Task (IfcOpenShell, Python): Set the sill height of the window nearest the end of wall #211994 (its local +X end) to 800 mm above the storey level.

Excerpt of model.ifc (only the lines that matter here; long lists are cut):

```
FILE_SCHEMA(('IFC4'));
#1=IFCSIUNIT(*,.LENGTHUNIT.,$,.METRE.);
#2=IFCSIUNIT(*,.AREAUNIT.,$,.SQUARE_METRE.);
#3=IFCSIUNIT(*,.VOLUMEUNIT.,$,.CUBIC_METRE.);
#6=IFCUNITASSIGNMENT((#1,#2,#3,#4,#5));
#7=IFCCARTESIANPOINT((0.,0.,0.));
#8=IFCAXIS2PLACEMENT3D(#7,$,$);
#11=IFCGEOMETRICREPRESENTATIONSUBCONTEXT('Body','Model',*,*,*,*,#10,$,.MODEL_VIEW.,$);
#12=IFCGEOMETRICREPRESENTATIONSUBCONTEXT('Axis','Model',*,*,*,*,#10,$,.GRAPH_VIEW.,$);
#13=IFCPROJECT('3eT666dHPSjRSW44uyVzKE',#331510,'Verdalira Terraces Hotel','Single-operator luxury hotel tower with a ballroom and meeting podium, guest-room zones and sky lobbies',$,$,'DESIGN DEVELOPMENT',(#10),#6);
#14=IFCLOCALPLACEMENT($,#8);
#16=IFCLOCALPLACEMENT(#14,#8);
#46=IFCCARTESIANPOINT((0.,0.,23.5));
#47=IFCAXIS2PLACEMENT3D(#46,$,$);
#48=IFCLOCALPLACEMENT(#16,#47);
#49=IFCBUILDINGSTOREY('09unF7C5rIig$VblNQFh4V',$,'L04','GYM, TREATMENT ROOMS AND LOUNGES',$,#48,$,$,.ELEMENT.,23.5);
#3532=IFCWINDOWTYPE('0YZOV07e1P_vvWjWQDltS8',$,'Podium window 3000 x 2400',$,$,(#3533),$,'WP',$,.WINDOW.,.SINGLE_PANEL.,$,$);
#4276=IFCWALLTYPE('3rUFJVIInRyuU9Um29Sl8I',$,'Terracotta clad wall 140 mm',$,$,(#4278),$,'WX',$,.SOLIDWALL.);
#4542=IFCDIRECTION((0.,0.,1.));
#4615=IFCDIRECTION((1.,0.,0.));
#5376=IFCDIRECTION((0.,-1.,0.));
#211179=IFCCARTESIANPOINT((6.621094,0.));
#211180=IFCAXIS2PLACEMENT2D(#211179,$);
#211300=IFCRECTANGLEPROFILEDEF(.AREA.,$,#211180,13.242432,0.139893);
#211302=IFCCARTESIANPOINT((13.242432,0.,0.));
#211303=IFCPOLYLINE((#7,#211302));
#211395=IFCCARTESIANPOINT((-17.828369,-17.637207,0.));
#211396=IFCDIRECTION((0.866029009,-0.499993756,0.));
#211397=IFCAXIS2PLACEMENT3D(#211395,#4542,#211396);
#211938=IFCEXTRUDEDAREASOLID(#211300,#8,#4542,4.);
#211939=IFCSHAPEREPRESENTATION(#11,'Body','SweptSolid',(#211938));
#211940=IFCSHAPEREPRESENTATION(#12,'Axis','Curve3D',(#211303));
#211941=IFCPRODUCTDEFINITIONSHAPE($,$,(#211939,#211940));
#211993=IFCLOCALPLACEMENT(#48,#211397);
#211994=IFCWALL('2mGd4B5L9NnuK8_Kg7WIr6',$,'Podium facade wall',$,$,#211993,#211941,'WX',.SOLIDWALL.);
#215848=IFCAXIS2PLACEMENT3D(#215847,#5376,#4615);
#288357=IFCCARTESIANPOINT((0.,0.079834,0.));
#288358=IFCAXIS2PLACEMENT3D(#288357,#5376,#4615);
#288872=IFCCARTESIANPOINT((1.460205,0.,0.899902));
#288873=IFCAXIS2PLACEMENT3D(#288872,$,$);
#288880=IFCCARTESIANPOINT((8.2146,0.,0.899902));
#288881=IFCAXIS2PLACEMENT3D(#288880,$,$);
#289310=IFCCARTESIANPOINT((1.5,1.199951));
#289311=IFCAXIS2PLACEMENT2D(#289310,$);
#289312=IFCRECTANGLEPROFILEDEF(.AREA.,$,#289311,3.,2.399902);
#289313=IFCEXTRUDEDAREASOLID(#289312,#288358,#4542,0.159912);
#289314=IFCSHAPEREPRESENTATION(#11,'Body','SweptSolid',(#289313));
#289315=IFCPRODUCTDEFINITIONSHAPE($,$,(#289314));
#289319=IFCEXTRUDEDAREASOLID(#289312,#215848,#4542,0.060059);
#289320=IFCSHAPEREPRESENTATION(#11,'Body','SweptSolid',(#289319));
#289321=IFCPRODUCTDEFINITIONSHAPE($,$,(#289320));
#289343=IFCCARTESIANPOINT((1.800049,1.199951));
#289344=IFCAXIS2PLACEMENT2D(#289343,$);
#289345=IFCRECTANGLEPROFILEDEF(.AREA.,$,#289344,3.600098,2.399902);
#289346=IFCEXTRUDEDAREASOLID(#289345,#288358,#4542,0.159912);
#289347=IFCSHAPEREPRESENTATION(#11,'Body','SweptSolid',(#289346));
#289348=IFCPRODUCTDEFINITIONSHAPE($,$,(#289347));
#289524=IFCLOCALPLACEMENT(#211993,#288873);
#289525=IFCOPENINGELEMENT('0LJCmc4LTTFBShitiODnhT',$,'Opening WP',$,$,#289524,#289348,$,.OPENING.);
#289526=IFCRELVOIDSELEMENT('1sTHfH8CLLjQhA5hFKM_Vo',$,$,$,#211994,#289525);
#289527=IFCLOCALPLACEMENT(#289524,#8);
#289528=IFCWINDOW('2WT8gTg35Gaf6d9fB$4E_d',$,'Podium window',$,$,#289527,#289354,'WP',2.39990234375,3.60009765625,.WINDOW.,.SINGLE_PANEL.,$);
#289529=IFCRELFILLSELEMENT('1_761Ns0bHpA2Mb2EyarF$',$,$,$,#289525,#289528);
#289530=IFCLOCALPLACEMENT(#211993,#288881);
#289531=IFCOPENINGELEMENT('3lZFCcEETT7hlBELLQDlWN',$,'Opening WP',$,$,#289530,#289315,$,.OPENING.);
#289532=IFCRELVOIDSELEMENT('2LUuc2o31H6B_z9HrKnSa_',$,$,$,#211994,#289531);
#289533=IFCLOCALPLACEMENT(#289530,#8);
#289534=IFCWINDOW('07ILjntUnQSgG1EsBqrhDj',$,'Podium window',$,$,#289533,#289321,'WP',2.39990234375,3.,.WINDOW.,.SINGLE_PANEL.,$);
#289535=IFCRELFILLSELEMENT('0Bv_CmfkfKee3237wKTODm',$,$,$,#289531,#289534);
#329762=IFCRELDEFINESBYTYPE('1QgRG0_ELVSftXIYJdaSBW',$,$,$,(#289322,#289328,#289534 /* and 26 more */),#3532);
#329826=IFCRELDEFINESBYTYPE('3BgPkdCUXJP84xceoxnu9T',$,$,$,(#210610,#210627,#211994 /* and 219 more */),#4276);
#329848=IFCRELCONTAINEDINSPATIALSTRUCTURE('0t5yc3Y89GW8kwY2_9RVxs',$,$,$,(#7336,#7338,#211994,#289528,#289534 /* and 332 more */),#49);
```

```python
import numpy as np
import ifcopenshell
import ifcopenshell.api.geometry
import ifcopenshell.geom
import ifcopenshell.util.element
import ifcopenshell.util.placement
import ifcopenshell.util.shape
import ifcopenshell.util.unit

model = ifcopenshell.open("model.ifc")
unit_scale = ifcopenshell.util.unit.calculate_unit_scale(model)

window = model.by_id(289534)
opening = window.FillsVoids[0].RelatingOpeningElement
storey = ifcopenshell.util.element.get_container(window, ifc_class="IfcBuildingStorey")
level = ifcopenshell.util.placement.get_local_placement(storey.ObjectPlacement)[2, 3]

# The opening's origin need not be at the sill, so measure its lowest point.
shape = ifcopenshell.geom.create_shape(ifcopenshell.geom.settings(), opening)
bottom = ifcopenshell.util.shape.get_shape_bottom_elevation(shape, shape.geometry) / unit_scale
dz = level + 0.8 - bottom

shift = np.array([0.0, 0.0, dz])
# The window is placed relative to its opening, so it follows when the opening moves.
matrix = ifcopenshell.util.placement.get_local_placement(opening.ObjectPlacement)
matrix[:3, 3] += shift
ifcopenshell.api.geometry.edit_object_placement(
    model, product=opening, matrix=matrix, is_si=False, should_transform_children=True
)

print(f"moved by {dz * unit_scale:+.3f} m")

model.write("model_rev.ifc")
```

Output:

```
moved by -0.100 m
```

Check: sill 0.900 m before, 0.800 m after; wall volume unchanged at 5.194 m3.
